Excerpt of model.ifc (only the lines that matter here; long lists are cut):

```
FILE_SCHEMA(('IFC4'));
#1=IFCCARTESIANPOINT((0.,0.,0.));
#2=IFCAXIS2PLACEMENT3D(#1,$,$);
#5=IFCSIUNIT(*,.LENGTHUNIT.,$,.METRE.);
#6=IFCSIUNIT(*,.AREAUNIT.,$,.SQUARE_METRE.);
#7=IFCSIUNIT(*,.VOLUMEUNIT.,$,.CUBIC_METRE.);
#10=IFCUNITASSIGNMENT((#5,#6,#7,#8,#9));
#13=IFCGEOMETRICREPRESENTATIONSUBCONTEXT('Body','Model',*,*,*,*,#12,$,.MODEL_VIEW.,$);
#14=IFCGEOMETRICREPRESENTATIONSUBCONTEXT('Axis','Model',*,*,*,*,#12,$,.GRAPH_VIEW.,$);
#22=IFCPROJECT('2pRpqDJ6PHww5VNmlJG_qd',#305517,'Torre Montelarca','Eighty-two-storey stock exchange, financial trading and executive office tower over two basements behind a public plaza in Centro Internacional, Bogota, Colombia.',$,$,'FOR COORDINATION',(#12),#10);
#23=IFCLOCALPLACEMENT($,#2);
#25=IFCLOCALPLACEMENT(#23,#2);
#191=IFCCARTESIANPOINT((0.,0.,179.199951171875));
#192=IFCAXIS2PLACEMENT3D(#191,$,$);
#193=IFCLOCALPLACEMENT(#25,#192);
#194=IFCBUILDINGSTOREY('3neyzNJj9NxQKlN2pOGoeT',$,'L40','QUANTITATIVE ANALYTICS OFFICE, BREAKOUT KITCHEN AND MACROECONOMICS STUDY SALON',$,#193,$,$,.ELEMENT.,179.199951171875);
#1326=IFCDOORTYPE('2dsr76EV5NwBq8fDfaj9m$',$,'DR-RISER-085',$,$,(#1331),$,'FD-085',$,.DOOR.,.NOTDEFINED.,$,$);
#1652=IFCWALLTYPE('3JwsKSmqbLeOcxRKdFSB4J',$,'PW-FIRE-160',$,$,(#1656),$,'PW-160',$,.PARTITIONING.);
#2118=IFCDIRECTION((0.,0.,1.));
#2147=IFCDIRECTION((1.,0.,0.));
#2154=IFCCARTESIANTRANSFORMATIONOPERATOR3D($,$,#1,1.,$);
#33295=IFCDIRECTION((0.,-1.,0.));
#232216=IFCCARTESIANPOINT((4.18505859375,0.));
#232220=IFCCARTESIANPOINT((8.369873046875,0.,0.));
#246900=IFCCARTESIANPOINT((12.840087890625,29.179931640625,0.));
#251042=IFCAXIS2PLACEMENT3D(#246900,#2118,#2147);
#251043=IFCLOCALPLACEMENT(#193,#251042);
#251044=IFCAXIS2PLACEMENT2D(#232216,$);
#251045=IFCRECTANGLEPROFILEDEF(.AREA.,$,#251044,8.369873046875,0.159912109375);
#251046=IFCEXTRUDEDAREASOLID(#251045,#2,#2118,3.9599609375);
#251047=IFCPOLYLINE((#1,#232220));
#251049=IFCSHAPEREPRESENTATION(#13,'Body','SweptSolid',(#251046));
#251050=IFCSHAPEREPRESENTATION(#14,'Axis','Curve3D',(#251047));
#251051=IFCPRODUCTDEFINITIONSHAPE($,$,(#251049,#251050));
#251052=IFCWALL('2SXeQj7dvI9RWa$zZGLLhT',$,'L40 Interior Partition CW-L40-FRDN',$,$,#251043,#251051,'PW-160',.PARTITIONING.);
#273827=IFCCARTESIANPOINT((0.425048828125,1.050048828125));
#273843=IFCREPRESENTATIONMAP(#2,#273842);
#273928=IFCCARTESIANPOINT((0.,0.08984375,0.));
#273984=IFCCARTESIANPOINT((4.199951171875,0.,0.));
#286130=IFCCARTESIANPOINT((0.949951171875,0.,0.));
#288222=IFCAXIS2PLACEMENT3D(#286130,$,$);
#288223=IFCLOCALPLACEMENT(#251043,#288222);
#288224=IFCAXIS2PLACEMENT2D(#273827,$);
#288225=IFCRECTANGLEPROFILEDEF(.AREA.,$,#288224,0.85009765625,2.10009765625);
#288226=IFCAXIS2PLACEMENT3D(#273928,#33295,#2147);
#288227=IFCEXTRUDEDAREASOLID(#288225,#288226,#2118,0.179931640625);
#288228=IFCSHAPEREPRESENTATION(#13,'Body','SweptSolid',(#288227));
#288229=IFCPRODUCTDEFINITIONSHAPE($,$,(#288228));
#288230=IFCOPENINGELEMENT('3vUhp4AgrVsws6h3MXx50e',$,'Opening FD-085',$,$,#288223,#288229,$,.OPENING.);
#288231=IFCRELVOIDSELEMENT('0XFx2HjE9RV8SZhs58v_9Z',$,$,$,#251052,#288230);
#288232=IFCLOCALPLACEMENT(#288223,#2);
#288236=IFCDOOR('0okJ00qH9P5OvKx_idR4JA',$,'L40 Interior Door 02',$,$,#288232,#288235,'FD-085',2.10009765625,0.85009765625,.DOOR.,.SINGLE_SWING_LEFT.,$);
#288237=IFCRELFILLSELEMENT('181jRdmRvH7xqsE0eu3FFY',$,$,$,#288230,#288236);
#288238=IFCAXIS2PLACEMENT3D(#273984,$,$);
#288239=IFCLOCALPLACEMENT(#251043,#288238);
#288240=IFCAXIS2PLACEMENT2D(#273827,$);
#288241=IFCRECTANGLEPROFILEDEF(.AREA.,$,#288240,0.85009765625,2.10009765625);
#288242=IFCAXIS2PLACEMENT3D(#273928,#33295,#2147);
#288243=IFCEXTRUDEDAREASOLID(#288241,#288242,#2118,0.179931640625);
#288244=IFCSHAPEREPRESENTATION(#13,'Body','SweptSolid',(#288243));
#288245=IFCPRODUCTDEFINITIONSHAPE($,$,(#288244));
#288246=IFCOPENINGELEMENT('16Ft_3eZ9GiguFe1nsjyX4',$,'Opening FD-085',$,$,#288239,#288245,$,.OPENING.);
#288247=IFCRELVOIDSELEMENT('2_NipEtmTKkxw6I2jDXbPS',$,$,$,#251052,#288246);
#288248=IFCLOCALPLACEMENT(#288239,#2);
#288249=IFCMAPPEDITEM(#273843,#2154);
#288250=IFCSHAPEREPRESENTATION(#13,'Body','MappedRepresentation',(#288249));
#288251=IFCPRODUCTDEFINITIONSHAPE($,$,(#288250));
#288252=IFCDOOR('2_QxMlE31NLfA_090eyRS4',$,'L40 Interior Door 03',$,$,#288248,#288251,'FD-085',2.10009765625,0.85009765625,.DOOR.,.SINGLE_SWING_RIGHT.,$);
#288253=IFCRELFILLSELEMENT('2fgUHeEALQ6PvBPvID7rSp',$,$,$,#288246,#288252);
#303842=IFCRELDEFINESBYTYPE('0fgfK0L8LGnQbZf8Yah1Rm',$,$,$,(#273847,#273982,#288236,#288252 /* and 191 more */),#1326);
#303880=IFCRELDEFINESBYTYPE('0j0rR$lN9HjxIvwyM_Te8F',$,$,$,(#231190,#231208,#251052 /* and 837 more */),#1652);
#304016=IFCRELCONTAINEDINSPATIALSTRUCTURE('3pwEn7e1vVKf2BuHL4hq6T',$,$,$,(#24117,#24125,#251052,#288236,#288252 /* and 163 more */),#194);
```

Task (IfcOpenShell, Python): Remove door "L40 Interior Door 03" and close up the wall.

```python
import ifcopenshell
import ifcopenshell.api.feature
import ifcopenshell.api.root
import ifcopenshell.geom
import ifcopenshell.util.shape

model = ifcopenshell.open("model.ifc")
settings = ifcopenshell.geom.settings()


def volume(element):
    """Net volume in cubic metres, openings subtracted."""
    shape = ifcopenshell.geom.create_shape(settings, element)
    return ifcopenshell.util.shape.get_volume(shape.geometry)


door = model.by_guid("2_QxMlE31NLfA_090eyRS4")
opening = door.FillsVoids[0].RelatingOpeningElement
wall = opening.VoidsElements[0].RelatingBuildingElement
before = volume(wall)

ifcopenshell.api.root.remove_product(model, product=door)
ifcopenshell.api.feature.remove_feature(model, feature=opening)

after = volume(wall)

print(f"wall volume {before:.3f} -> {after:.3f} m3")

model.write("model_v2.ifc")
```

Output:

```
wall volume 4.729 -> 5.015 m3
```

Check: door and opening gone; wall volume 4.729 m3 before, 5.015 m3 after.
